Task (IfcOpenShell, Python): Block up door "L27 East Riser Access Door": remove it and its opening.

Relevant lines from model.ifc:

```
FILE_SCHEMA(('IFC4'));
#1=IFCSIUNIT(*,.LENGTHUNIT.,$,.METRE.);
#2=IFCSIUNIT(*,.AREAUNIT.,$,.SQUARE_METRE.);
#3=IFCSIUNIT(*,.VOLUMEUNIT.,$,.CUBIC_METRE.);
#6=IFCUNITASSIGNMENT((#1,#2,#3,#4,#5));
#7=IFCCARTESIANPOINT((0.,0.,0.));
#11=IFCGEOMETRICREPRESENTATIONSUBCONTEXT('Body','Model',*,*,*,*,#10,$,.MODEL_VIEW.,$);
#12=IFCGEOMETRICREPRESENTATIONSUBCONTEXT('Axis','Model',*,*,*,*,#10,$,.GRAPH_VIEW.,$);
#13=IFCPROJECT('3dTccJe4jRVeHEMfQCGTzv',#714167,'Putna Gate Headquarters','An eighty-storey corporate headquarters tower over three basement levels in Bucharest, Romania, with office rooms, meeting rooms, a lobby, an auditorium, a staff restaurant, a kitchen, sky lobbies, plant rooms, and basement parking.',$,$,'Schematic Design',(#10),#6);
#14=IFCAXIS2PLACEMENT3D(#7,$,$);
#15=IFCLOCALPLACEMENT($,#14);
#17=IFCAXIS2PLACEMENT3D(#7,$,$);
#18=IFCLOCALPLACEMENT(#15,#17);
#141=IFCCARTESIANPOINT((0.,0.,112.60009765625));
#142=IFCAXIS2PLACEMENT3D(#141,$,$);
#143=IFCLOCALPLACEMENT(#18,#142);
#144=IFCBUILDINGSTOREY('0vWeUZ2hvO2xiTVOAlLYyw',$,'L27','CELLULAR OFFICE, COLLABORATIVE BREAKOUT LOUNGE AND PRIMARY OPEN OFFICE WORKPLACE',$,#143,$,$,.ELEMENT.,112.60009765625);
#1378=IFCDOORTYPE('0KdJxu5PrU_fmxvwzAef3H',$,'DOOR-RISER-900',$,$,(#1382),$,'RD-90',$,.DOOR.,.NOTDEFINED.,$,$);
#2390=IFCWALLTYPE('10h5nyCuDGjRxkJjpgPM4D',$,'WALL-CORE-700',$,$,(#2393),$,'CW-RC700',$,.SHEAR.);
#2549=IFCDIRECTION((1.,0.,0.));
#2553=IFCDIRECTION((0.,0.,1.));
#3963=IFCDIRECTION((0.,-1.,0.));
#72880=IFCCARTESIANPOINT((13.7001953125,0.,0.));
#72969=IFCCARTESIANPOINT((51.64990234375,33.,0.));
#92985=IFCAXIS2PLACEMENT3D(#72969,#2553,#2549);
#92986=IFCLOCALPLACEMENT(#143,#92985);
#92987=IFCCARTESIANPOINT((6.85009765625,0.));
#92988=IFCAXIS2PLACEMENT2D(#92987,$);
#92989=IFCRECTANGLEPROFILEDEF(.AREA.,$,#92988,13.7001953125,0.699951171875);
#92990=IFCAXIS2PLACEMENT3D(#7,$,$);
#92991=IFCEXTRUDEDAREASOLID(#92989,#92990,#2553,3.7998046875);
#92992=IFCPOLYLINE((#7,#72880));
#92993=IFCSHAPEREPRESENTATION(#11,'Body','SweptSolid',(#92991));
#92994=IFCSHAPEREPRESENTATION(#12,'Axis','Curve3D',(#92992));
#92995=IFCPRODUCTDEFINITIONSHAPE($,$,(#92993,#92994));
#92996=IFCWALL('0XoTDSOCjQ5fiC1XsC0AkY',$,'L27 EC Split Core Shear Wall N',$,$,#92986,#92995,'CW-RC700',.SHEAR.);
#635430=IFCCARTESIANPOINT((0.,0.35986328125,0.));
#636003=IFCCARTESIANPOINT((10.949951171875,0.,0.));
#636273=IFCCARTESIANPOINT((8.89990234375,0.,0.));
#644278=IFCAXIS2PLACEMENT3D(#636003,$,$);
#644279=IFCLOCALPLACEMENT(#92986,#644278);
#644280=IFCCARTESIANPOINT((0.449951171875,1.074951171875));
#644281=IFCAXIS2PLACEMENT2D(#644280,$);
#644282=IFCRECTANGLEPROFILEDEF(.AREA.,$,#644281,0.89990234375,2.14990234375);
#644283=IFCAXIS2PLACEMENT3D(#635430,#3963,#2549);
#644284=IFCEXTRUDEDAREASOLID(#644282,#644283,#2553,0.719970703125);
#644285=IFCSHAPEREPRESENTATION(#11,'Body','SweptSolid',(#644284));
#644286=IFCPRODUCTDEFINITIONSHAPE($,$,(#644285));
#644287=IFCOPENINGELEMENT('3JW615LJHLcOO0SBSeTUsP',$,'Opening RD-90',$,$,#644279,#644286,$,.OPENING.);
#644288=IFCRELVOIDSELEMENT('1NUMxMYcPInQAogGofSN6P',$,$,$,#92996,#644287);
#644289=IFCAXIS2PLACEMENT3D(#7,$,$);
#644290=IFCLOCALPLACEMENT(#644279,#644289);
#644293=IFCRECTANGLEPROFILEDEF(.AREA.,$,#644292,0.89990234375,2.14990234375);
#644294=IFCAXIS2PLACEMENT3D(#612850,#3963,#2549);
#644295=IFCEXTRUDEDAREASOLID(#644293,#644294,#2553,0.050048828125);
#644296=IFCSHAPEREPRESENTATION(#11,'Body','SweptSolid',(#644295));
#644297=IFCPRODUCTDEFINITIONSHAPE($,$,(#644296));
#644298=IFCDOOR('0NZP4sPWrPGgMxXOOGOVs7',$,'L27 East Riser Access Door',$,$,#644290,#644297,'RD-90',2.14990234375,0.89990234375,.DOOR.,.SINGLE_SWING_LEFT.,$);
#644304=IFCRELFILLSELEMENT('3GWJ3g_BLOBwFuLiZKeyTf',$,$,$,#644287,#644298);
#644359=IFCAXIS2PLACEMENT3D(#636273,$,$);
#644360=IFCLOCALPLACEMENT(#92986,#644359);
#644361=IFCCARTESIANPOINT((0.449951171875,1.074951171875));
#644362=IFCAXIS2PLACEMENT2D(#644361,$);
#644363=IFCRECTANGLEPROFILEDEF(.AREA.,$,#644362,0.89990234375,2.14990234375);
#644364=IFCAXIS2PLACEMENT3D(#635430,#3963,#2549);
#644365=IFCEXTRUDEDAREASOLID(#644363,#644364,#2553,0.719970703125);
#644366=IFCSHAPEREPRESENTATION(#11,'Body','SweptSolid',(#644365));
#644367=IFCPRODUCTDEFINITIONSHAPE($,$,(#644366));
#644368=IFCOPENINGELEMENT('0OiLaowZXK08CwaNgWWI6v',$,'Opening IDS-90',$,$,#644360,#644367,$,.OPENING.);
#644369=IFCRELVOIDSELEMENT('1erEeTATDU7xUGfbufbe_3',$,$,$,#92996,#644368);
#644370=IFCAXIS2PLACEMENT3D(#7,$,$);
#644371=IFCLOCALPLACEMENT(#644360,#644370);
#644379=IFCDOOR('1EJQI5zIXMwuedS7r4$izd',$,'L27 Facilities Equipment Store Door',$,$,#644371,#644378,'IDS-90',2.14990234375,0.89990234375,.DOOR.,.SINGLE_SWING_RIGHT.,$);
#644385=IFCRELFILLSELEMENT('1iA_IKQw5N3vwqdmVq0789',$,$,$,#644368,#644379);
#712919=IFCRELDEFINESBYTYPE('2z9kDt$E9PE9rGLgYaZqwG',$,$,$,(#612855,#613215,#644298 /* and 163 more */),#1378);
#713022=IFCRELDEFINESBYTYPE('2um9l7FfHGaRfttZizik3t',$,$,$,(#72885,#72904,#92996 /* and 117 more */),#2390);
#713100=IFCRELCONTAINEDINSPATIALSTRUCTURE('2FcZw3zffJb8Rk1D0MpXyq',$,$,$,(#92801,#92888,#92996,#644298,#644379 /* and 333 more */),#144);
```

```python
import ifcopenshell
import ifcopenshell.api.feature
import ifcopenshell.api.root
import ifcopenshell.geom
import ifcopenshell.util.shape

model = ifcopenshell.open("model.ifc")
settings = ifcopenshell.geom.settings()


def volume(element):
    """Net volume in cubic metres, openings subtracted."""
    shape = ifcopenshell.geom.create_shape(settings, element)
    return ifcopenshell.util.shape.get_volume(shape.geometry)


door = model.by_guid("0NZP4sPWrPGgMxXOOGOVs7")
opening = door.FillsVoids[0].RelatingOpeningElement
wall = opening.VoidsElements[0].RelatingBuildingElement
before = volume(wall)

ifcopenshell.api.root.remove_product(model, product=door)
ifcopenshell.api.feature.remove_feature(model, feature=opening)

after = volume(wall)

print(f"wall volume {before:.3f} -> {after:.3f} m3")

model.write("model_rev.ifc")
```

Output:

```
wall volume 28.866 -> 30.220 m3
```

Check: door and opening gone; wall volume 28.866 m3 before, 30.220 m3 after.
